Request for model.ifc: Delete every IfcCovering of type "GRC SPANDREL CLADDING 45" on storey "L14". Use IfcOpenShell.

First a look at what the model holds.

```python
import ifcopenshell
import ifcopenshell.util.element

model = ifcopenshell.open("model.ifc")
print(model.schema)
storey = next(s for s in model.by_type("IfcBuildingStorey") if s.Name == "L14")
coverings = [e for e in ifcopenshell.util.element.get_decomposition(storey) if e.is_a("IfcCovering")]
seen = {}
for e in coverings:
    element_type = ifcopenshell.util.element.get_type(e)
    name = element_type.Name if element_type not in (None, e) else None
    seen[name] = seen.get(name, 0) + 1
for name, count in sorted(seen.items(), key=str):
    print(count, "x", name)
```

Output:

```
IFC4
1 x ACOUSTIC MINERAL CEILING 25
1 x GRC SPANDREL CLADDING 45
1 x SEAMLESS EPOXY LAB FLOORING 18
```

```python
import ifcopenshell
import ifcopenshell.api.root
import ifcopenshell.util.element

model = ifcopenshell.open("model.ifc")

storey = next(s for s in model.by_type("IfcBuildingStorey") if s.Name == "L14")
coverings = [e for e in ifcopenshell.util.element.get_decomposition(storey) if e.is_a("IfcCovering")]
targets = [e for e in coverings if (t := ifcopenshell.util.element.get_type(e)) not in (None, e) and t.Name == "GRC SPANDREL CLADDING 45"]

for e in targets:
    ifcopenshell.api.root.remove_product(model, product=e)
print(len(targets), "removed")

model.write("model-out.ifc")
```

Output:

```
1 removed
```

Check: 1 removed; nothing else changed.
